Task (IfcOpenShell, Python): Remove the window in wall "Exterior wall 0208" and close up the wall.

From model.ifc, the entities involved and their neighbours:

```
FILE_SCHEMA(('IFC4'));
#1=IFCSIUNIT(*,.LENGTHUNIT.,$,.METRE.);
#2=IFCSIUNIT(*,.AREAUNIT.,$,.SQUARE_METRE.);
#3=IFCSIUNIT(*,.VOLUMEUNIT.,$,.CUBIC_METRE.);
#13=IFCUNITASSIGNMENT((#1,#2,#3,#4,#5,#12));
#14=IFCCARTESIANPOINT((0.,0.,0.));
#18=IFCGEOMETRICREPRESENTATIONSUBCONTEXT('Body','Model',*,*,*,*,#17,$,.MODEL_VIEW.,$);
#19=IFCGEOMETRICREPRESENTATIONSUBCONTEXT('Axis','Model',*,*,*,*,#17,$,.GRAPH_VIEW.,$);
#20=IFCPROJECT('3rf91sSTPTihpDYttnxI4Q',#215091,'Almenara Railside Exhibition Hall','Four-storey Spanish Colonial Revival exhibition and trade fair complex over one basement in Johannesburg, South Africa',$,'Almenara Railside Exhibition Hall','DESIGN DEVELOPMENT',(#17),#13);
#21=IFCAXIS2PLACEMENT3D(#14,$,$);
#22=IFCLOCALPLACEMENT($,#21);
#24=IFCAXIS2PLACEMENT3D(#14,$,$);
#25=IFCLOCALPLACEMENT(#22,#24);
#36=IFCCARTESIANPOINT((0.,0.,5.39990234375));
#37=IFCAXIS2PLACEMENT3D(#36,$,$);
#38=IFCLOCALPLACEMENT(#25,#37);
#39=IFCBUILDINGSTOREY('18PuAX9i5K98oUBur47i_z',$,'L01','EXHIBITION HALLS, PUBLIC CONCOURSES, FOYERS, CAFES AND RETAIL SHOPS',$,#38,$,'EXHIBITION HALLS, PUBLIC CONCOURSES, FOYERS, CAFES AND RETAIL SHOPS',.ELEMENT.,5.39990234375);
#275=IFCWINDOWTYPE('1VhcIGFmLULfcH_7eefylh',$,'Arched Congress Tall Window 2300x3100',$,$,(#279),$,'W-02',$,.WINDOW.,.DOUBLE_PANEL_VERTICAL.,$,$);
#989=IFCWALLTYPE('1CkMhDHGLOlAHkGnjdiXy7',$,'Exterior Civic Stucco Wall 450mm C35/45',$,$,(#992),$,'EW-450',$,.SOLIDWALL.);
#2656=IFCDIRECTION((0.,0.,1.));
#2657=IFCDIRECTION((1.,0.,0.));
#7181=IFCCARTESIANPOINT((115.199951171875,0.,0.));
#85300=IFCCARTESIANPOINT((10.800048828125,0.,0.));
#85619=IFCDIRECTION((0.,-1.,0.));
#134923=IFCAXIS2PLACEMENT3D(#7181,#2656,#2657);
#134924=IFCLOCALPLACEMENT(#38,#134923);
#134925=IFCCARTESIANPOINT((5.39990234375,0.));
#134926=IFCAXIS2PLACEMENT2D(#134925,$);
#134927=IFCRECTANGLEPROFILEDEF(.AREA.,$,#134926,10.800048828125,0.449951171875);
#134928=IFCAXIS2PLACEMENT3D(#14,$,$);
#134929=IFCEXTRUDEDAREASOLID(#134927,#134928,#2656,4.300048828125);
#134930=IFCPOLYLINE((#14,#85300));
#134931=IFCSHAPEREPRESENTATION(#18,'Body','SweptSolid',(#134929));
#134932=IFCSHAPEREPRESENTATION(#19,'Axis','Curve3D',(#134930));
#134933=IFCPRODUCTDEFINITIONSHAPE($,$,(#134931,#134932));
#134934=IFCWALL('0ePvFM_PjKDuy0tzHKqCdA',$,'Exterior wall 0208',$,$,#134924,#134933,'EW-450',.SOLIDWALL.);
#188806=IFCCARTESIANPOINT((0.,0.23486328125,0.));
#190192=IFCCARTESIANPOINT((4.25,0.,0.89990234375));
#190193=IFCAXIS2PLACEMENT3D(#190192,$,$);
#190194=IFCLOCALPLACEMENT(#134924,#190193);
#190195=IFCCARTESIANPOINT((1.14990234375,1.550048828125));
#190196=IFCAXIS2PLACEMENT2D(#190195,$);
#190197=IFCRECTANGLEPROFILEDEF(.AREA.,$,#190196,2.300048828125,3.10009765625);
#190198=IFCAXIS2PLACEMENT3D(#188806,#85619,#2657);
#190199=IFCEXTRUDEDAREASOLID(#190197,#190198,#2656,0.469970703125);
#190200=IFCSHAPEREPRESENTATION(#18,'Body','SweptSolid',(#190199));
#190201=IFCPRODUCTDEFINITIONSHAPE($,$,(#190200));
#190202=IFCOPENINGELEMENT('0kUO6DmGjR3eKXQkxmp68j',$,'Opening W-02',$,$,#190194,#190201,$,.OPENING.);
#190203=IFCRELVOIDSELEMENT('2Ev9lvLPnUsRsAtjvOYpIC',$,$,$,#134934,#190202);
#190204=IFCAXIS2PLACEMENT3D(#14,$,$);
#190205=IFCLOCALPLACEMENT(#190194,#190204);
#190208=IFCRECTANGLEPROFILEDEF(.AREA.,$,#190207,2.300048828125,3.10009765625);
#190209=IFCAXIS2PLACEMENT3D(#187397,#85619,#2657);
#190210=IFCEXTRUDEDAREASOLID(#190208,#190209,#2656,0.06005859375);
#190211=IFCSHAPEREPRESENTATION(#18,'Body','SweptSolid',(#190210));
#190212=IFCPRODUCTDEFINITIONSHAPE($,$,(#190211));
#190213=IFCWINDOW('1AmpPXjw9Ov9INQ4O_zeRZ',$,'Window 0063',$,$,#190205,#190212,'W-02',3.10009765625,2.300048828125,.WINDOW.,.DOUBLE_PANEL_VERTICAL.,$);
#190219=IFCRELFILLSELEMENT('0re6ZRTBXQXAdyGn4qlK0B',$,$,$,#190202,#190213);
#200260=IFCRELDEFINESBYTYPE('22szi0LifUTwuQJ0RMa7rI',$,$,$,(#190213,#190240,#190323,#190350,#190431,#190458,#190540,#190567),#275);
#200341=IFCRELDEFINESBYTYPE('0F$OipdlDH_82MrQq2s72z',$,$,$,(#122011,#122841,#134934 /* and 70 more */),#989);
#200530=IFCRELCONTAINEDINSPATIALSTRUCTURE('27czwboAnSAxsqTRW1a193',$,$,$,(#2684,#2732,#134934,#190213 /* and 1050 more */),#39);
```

```python
import ifcopenshell
import ifcopenshell.api.feature
import ifcopenshell.api.root
import ifcopenshell.geom
import ifcopenshell.util.shape

model = ifcopenshell.open("model.ifc")
settings = ifcopenshell.geom.settings()


def volume(element):
    """Net volume in cubic metres, openings subtracted."""
    shape = ifcopenshell.geom.create_shape(settings, element)
    return ifcopenshell.util.shape.get_volume(shape.geometry)


window = model.by_guid("1AmpPXjw9Ov9INQ4O_zeRZ")
opening = window.FillsVoids[0].RelatingOpeningElement
wall = opening.VoidsElements[0].RelatingBuildingElement
before = volume(wall)

ifcopenshell.api.root.remove_product(model, product=window)
ifcopenshell.api.feature.remove_feature(model, feature=opening)

after = volume(wall)

print(f"wall volume {before:.3f} -> {after:.3f} m3")

model.write("model_rev.ifc")
```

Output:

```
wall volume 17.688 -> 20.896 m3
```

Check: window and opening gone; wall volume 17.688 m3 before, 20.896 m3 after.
